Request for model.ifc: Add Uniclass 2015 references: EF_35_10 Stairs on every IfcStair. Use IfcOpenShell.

First a look at what the model holds.

```python
import ifcopenshell

model = ifcopenshell.open("model.ifc")
print(model.schema)
print("classifications:", [c.Name for c in model.by_type("IfcClassification")])
for ifc_class in ("IfcDoor", "IfcRoof", "IfcStair", "IfcWall", "IfcWindow"):
    print(ifc_class, len(model.by_type(ifc_class)))
```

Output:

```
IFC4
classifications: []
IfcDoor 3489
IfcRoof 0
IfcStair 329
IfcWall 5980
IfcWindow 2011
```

```python
import ifcopenshell
import ifcopenshell.api.classification

model = ifcopenshell.open("model.ifc")

system = ifcopenshell.api.classification.add_classification(model, classification="Uniclass 2015")

codes = {
    "IfcStair": ("EF_35_10", "Stairs"),
}
for ifc_class, (code, name) in codes.items():
    products = model.by_type(ifc_class)
    ifcopenshell.api.classification.add_reference(
        model, products=products, classification=system, identification=code, name=name
    )
    print(code, len(products))

model.write("model_v2.ifc")
```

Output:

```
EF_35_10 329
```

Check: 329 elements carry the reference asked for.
